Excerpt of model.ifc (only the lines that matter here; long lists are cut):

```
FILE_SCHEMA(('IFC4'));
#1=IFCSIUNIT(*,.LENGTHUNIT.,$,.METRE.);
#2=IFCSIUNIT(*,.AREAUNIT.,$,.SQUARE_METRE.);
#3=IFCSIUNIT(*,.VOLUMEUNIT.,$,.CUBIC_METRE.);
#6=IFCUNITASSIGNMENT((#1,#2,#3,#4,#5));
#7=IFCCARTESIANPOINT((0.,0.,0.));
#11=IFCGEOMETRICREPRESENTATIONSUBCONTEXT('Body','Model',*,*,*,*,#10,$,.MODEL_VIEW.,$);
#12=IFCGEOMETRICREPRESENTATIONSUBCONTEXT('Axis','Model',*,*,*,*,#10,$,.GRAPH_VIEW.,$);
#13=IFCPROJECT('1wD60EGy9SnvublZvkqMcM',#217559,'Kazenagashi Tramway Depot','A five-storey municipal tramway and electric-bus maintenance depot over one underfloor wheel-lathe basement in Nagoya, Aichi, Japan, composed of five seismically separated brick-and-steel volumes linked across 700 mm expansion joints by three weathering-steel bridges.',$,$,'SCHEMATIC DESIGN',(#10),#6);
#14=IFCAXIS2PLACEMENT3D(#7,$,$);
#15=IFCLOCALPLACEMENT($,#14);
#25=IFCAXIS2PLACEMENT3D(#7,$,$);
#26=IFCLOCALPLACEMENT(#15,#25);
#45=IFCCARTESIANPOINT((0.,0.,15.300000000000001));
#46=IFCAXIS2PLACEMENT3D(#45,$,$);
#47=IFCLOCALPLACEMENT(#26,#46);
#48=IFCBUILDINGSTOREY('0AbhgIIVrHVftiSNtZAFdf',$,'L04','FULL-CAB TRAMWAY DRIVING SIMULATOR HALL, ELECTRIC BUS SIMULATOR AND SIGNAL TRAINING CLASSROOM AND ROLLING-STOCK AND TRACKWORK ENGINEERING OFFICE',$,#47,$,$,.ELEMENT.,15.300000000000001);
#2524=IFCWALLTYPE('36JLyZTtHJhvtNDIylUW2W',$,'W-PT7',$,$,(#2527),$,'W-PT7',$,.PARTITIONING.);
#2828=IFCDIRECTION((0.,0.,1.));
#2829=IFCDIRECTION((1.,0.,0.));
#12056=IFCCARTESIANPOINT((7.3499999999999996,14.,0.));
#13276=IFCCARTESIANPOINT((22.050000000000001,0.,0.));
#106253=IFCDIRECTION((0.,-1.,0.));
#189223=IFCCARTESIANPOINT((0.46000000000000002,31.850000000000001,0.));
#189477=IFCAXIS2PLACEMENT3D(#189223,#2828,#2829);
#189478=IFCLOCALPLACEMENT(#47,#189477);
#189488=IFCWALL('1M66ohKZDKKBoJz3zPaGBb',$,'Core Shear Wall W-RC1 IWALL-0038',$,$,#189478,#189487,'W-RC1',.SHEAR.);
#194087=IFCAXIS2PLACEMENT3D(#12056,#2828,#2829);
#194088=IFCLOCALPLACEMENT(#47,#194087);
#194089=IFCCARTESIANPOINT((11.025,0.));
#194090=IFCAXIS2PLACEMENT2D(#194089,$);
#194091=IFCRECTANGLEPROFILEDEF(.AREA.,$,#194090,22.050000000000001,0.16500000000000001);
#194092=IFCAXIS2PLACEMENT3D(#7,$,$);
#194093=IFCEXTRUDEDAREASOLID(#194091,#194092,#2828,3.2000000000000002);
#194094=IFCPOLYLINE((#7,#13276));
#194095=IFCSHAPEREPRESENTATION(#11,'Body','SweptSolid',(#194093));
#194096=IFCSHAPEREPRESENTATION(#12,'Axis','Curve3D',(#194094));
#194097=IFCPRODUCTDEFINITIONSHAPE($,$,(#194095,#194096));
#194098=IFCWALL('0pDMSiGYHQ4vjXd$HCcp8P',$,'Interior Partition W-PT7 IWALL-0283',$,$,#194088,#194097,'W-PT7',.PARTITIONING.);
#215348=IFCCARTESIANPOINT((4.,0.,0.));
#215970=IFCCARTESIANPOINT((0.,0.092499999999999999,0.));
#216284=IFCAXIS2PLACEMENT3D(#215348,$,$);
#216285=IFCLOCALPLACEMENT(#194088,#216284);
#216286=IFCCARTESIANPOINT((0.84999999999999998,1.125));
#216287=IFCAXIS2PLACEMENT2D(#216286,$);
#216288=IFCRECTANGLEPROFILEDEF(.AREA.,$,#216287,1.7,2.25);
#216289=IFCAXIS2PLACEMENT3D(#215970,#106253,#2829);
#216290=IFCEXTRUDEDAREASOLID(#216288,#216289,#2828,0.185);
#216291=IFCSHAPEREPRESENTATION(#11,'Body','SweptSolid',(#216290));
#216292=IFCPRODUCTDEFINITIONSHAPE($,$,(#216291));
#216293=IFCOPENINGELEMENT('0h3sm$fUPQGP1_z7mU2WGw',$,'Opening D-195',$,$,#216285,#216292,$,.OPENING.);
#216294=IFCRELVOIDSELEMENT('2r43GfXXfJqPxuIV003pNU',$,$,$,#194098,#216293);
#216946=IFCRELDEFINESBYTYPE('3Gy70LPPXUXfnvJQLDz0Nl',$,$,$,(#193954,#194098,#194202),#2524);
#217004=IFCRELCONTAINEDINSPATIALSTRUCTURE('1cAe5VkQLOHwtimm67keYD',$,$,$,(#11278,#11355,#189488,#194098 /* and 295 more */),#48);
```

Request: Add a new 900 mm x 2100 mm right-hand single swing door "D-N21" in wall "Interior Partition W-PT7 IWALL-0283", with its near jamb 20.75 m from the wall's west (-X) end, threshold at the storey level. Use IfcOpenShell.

```python
import numpy as np
import ifcopenshell
import ifcopenshell.api.feature
import ifcopenshell.api.geometry
import ifcopenshell.api.root
import ifcopenshell.api.spatial
import ifcopenshell.geom
import ifcopenshell.util.element
import ifcopenshell.util.placement
import ifcopenshell.util.representation
import ifcopenshell.util.shape
import ifcopenshell.util.unit

model = ifcopenshell.open("model.ifc")
unit_scale = ifcopenshell.util.unit.calculate_unit_scale(model)
settings = ifcopenshell.geom.settings()


def volume(element):
    """Net volume in cubic metres, openings subtracted."""
    shape = ifcopenshell.geom.create_shape(settings, element)
    return ifcopenshell.util.shape.get_volume(shape.geometry)


wall = model.by_id(194098)
storey = ifcopenshell.util.element.get_container(wall, ifc_class="IfcBuildingStorey")
context = ifcopenshell.util.representation.get_context(model, "Model", "Body", "MODEL_VIEW")
before = volume(wall)

width, height, from_end, sill = 0.9, 2.1, 20.75, 0.0  # metres

# The wall runs along its own X axis, and the end named is its -X end.
wall_shape = ifcopenshell.geom.create_shape(settings, wall)
x, y, z = ifcopenshell.util.shape.get_vertices(wall_shape.geometry).T
start = x.min() + from_end
face, thickness = float(y.min()), float(y.max() - y.min())
wall_matrix = ifcopenshell.util.placement.get_local_placement(wall.ObjectPlacement)
level = ifcopenshell.util.placement.get_local_placement(storey.ObjectPlacement)[2, 3]


def in_wall(x, y):
    """Placement at x, y metres in the wall's axes, at sill height."""
    matrix = wall_matrix.copy()
    matrix[:, 3] = wall_matrix @ np.array([x / unit_scale, y / unit_scale, 0.0, 1.0])
    matrix[2, 3] = level + sill / unit_scale
    return matrix


# Opening: a box that overshoots both wall faces by 50 mm.
opening = ifcopenshell.api.root.create_entity(model, ifc_class="IfcOpeningElement", predefined_type="OPENING")
box = ifcopenshell.api.geometry.add_wall_representation(
    model, context=context, length=width, height=height, thickness=thickness + 0.1
)
ifcopenshell.api.geometry.assign_representation(model, product=opening, representation=box)
ifcopenshell.api.geometry.edit_object_placement(model, product=opening, matrix=in_wall(start, face - 0.05), is_si=False)
ifcopenshell.api.feature.add_feature(model, feature=opening, element=wall)

door = ifcopenshell.api.root.create_entity(model, ifc_class="IfcDoor", name="D-N21", predefined_type="DOOR")
door.OverallWidth, door.OverallHeight = width / unit_scale, height / unit_scale
door.OperationType = "SINGLE_SWING_RIGHT"
body = ifcopenshell.api.geometry.add_door_representation(
    model,
    context=context,
    overall_width=door.OverallWidth,
    overall_height=door.OverallHeight,
    operation_type="SINGLE_SWING_RIGHT",
    lining_properties={"LiningDepth": thickness / unit_scale, "ThresholdDepth": thickness / unit_scale},
)
ifcopenshell.api.geometry.assign_representation(model, product=door, representation=body)
ifcopenshell.api.spatial.assign_container(model, products=[door], relating_structure=storey)
ifcopenshell.api.feature.add_filling(model, opening=opening, element=door)

# The lining spans the wall, so the door starts at the wall face.
ifcopenshell.api.geometry.edit_object_placement(model, product=door, matrix=in_wall(start, face), is_si=False)

after = volume(wall)

print(f"wall volume {before:.3f} -> {after:.3f} m3")

model.write("model-out.ifc")
```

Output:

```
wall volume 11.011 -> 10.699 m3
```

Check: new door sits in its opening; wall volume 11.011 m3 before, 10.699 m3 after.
